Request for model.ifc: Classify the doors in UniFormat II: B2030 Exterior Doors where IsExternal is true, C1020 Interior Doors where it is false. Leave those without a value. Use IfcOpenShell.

First a look at what the model holds.

```python
import ifcopenshell
import ifcopenshell.util.element

model = ifcopenshell.open("model.ifc")
print(model.schema)
print("classifications:", [c.Name for c in model.by_type("IfcClassification")])
values = [ifcopenshell.util.element.get_pset(e, "Pset_DoorCommon", "IsExternal") for e in model.by_type("IfcDoor")]
for value in (True, False, None):
    print("IsExternal", value, values.count(value))
```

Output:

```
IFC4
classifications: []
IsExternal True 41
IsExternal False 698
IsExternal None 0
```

```python
import ifcopenshell
import ifcopenshell.api.classification
import ifcopenshell.util.element

model = ifcopenshell.open("model.ifc")

system = ifcopenshell.api.classification.add_classification(model, classification="UniFormat II")

doors = model.by_type("IfcDoor")
external = {e: ifcopenshell.util.element.get_pset(e, "Pset_DoorCommon", "IsExternal") for e in doors}
for flag, code, name in ((True, "B2030", "Exterior Doors"), (False, "C1020", "Interior Doors")):
    products = [e for e in doors if external[e] is flag]
    ifcopenshell.api.classification.add_reference(
        model, products=products, classification=system, identification=code, name=name
    )
    print(code, len(products))

model.write("model_edited.ifc")
```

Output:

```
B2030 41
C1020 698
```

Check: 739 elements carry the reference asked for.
